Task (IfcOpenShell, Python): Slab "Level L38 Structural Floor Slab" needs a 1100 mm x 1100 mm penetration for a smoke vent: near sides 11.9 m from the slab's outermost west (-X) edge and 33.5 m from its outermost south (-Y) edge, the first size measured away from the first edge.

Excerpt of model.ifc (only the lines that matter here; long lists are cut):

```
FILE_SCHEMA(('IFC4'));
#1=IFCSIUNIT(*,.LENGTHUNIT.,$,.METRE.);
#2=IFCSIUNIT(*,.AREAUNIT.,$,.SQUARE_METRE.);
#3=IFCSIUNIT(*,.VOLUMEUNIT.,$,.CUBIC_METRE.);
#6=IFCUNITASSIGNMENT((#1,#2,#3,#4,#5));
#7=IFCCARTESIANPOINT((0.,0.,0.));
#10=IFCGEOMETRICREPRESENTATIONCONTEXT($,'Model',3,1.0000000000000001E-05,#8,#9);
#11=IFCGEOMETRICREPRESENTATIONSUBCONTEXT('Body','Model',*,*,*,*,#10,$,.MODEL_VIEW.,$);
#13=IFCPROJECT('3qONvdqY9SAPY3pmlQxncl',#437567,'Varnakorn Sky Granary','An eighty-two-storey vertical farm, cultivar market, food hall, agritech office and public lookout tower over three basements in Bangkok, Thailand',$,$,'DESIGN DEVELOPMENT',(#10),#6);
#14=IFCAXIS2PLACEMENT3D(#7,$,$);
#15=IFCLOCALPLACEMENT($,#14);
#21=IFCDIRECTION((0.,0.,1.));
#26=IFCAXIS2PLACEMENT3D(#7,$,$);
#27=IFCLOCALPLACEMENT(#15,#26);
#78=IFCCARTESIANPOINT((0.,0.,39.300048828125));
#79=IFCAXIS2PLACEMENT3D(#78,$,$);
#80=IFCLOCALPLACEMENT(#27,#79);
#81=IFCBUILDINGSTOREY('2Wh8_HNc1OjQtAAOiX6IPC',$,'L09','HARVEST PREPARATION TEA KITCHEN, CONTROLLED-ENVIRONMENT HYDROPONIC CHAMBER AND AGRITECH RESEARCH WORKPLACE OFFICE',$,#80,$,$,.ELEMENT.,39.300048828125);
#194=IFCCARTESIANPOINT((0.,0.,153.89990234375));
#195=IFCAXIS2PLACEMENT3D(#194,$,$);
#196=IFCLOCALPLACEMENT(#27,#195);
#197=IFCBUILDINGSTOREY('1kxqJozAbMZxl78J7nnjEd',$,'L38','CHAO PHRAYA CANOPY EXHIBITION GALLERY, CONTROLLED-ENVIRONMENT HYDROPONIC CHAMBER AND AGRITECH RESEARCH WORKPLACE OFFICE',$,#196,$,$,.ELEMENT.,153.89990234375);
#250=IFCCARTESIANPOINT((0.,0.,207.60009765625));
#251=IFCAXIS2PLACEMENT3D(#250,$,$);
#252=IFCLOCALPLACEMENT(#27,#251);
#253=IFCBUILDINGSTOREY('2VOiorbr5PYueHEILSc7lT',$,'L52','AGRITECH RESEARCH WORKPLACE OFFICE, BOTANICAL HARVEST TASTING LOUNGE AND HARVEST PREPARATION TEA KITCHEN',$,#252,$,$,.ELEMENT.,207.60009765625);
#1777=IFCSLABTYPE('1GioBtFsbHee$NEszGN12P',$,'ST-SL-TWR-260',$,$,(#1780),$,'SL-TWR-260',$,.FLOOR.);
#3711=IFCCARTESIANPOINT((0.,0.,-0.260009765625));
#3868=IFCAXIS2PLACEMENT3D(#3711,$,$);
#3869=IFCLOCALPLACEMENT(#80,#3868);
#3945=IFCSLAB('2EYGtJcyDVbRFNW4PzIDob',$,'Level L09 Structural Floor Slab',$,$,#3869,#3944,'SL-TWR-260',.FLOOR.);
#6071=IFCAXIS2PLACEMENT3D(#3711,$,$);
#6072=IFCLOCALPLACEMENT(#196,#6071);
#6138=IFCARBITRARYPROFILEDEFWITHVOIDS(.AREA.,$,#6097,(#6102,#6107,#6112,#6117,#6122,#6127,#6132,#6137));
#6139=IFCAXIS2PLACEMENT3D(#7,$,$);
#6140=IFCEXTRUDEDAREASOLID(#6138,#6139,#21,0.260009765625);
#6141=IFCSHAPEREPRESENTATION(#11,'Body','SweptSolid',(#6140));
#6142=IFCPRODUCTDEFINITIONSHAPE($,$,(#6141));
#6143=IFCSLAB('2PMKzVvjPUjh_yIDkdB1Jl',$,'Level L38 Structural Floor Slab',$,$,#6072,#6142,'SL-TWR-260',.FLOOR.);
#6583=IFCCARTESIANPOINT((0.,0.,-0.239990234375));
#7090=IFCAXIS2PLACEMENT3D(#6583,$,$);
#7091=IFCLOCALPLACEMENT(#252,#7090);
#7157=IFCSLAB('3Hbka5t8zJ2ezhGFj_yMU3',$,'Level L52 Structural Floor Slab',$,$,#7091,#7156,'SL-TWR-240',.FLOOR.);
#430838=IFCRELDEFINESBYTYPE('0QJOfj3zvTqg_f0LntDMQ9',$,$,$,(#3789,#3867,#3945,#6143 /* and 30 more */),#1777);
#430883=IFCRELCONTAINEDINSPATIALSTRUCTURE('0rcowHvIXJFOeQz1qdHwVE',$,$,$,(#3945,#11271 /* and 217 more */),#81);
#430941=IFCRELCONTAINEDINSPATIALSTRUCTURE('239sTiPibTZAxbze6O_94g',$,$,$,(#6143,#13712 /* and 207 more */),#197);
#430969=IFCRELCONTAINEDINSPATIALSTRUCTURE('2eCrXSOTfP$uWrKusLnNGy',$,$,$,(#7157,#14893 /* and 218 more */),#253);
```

```python
import numpy as np
import ifcopenshell
import ifcopenshell.api.feature
import ifcopenshell.api.geometry
import ifcopenshell.api.root
import ifcopenshell.geom
import ifcopenshell.util.placement
import ifcopenshell.util.representation
import ifcopenshell.util.shape
import ifcopenshell.util.unit

model = ifcopenshell.open("model.ifc")
unit_scale = ifcopenshell.util.unit.calculate_unit_scale(model)
settings = ifcopenshell.geom.settings()


def volume(element):
    """Net volume in cubic metres, openings subtracted."""
    shape = ifcopenshell.geom.create_shape(settings, element)
    return ifcopenshell.util.shape.get_volume(shape.geometry)


slab = model.by_guid("2PMKzVvjPUjh_yIDkdB1Jl")
before = volume(slab)

# Extent in the slab's own axes, in metres. The edges named are its -X and -Y sides.
slab_shape = ifcopenshell.geom.create_shape(settings, slab)
vertices = ifcopenshell.util.shape.get_vertices(slab_shape.geometry)
x_min, y_min, bottom = vertices.min(axis=0)
top = vertices[:, 2].max()

opening = ifcopenshell.api.root.create_entity(model, ifc_class="IfcOpeningElement", name="Smoke vent opening", predefined_type="OPENING")
context = ifcopenshell.util.representation.get_context(model, "Model", "Body", "MODEL_VIEW")
width, depth = 1.1, 1.1
outline = [(0.0, 0.0), (width, 0.0), (width, depth), (0.0, depth), (0.0, 0.0)]
# Overshoot both faces by 50 mm so the cut is clean.
shape = ifcopenshell.api.geometry.add_slab_representation(
    model, context=context, depth=top - bottom + 0.1, polyline=outline
)
ifcopenshell.api.geometry.assign_representation(model, product=opening, representation=shape)

matrix = ifcopenshell.util.placement.get_local_placement(slab.ObjectPlacement)
matrix[:, 3] = matrix @ np.append(np.array([x_min + 11.9, y_min + 33.5, bottom - 0.05]) / unit_scale, 1.0)
ifcopenshell.api.geometry.edit_object_placement(model, product=opening, matrix=matrix, is_si=False)
ifcopenshell.api.feature.add_feature(model, feature=opening, element=slab)

after = volume(slab)

print(f"slab volume {before:.3f} -> {after:.3f} m3")

model.write("model-out.ifc")
```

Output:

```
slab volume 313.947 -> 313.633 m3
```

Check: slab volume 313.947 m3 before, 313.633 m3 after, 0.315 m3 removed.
